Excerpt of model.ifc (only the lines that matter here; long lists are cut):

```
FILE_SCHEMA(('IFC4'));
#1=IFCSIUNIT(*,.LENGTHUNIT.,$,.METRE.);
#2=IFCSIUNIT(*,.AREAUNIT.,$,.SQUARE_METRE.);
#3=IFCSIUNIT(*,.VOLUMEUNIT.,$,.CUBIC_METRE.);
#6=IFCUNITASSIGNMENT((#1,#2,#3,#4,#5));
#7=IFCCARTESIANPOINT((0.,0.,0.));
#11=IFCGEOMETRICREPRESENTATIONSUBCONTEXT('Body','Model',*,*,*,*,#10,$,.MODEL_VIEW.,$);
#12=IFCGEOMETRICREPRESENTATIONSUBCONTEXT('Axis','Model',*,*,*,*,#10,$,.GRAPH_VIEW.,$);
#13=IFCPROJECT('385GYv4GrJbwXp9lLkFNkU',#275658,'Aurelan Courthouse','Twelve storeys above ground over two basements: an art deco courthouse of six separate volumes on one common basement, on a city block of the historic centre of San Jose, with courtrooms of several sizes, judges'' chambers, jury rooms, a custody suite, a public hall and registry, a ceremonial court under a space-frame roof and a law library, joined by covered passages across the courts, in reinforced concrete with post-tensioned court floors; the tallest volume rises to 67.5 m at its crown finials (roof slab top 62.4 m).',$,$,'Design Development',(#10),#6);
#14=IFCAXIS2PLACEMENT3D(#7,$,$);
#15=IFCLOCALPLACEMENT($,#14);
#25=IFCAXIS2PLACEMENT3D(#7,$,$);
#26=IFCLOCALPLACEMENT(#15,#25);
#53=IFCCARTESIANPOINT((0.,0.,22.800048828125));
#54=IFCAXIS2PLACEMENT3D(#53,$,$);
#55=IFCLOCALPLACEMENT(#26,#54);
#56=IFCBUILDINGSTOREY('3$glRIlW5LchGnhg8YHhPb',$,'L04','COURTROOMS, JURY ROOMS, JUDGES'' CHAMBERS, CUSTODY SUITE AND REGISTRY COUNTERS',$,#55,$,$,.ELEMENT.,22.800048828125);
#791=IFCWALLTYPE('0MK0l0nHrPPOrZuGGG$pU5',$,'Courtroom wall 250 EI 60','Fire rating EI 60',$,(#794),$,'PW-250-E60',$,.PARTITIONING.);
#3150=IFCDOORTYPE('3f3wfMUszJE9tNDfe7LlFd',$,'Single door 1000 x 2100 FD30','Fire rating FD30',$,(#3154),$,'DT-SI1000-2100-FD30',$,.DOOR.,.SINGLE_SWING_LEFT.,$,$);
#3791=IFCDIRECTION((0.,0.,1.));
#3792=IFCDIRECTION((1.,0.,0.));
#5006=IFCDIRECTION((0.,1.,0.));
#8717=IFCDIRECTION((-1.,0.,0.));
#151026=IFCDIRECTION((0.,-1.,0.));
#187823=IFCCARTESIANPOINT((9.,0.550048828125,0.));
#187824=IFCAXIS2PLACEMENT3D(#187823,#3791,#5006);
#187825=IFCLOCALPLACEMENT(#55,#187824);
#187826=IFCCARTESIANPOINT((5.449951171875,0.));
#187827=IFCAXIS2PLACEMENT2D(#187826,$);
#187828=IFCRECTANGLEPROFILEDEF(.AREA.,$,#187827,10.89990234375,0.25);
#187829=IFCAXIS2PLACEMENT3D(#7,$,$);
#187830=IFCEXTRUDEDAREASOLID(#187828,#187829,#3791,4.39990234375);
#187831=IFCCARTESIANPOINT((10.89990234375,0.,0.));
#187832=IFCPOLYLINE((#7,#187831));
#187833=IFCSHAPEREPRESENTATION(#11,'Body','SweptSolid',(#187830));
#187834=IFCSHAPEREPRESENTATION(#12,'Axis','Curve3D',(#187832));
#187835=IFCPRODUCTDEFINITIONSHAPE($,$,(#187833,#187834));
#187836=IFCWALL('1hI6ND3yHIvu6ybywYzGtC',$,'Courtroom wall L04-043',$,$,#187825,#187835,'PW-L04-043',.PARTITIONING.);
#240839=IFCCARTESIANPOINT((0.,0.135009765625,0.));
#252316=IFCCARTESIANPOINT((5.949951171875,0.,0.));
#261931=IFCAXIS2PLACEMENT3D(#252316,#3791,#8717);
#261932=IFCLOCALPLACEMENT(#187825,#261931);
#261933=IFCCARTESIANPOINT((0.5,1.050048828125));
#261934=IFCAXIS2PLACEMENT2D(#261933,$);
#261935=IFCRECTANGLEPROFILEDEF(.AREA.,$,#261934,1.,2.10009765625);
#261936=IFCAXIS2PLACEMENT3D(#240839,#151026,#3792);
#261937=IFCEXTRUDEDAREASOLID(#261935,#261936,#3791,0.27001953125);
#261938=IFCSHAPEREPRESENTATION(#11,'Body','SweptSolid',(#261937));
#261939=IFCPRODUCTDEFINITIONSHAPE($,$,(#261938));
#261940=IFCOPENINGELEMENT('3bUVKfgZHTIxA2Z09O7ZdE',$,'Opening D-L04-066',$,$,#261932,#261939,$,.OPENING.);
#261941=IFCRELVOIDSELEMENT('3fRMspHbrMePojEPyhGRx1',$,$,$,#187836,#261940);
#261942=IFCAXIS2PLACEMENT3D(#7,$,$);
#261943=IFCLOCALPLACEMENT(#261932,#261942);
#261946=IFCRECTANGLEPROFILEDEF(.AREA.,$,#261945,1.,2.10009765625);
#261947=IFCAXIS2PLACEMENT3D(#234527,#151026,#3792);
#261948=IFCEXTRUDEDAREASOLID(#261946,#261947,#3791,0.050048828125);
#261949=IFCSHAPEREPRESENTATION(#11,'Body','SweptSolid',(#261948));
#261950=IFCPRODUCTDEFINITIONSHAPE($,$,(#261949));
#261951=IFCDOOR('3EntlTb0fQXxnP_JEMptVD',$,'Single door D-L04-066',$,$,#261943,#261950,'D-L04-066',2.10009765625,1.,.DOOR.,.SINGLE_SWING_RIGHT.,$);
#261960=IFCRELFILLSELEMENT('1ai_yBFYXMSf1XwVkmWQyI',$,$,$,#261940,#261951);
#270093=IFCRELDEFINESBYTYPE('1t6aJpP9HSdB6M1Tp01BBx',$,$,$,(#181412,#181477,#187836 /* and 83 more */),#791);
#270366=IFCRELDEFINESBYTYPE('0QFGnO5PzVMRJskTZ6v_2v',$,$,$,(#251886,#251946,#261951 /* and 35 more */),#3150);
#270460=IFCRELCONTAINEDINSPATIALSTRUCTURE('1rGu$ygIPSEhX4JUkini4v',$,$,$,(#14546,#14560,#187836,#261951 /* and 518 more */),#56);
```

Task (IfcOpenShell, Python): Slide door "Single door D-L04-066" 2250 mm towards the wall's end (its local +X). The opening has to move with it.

```python
import ifcopenshell
import ifcopenshell.api.geometry
import ifcopenshell.util.placement

model = ifcopenshell.open("model.ifc")

door = model.by_guid("3EntlTb0fQXxnP_JEMptVD")
opening = door.FillsVoids[0].RelatingOpeningElement
wall = opening.VoidsElements[0].RelatingBuildingElement

wall_matrix = ifcopenshell.util.placement.get_local_placement(wall.ObjectPlacement)
shift = wall_matrix[:3, 0] * 2.25
before = ifcopenshell.util.placement.get_local_placement(door.ObjectPlacement)[:3, 3].copy()

# The door is placed relative to its opening, so it follows when the opening moves.
matrix = ifcopenshell.util.placement.get_local_placement(opening.ObjectPlacement)
matrix[:3, 3] += shift
ifcopenshell.api.geometry.edit_object_placement(
    model, product=opening, matrix=matrix, is_si=False, should_transform_children=True
)

after = ifcopenshell.util.placement.get_local_placement(door.ObjectPlacement)[:3, 3]
print("door moved by", (after - before).round(3) + 0.0)

model.write("model_v2.ifc")
```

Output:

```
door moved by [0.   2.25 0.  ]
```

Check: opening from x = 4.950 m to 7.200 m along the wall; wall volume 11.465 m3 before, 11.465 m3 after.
